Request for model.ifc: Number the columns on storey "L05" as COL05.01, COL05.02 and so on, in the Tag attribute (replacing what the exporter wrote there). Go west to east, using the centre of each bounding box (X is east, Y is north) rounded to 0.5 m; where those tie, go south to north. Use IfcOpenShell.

First a look at what the model holds.

```python
import ifcopenshell
import ifcopenshell.util.element
import ifcopenshell.util.placement

model = ifcopenshell.open("model.ifc")
print(model.schema)
storey = next(s for s in model.by_type("IfcBuildingStorey") if s.Name == "L05")
columns = [e for e in ifcopenshell.util.element.get_decomposition(storey) if e.is_a("IfcColumn")]
for e in sorted(columns, key=lambda e: e.id()):
    origin = ifcopenshell.util.placement.get_local_placement(e.ObjectPlacement)[:3, 3]
    print(e.id(), e.Tag, e.Name, origin.round(2) + 0.0, sep=" | ")
```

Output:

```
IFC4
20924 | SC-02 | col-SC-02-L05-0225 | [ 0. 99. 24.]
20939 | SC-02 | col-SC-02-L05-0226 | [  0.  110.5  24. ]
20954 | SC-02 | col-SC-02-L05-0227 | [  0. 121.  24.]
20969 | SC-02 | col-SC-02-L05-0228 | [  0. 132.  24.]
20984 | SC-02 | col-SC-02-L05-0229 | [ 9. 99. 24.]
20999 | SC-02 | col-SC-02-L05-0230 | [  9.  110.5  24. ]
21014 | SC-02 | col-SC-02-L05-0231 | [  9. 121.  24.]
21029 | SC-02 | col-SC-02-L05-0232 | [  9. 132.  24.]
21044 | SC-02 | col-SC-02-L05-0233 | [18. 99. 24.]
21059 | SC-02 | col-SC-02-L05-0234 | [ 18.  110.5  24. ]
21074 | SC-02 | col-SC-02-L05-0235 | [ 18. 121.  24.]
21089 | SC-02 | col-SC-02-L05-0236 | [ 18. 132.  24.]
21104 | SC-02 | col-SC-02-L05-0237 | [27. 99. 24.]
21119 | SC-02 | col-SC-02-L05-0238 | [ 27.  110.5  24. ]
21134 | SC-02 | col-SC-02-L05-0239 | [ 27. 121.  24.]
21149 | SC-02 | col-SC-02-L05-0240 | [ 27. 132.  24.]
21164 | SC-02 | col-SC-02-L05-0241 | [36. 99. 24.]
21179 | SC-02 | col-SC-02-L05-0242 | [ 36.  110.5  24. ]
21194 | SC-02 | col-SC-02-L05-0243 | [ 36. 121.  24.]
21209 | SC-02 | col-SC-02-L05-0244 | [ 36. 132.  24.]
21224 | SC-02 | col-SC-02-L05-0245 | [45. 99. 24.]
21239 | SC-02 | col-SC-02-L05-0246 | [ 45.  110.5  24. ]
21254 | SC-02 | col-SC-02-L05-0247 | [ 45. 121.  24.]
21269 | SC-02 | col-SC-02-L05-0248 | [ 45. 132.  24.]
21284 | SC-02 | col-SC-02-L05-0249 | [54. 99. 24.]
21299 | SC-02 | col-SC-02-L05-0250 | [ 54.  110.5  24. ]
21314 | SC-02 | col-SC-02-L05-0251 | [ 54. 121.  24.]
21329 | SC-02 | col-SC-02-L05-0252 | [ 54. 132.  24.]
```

```python
import ifcopenshell
import ifcopenshell.geom
import ifcopenshell.util.element
import ifcopenshell.util.shape

model = ifcopenshell.open("model.ifc")
settings = ifcopenshell.geom.settings()
settings.set("use-world-coords", True)


def centre(element):
    shape = ifcopenshell.geom.create_shape(settings, element)
    return ifcopenshell.util.shape.get_bbox_centroid(shape.geometry)


storey = next(s for s in model.by_type("IfcBuildingStorey") if s.Name == "L05")
columns = [e for e in ifcopenshell.util.element.get_decomposition(storey) if e.is_a("IfcColumn")]

# Insertion points can sit at a corner or the storey origin, so sort by the geometry (in metres).
centres = {e: centre(e) for e in columns}
columns.sort(key=lambda e: (round(centres[e][0] / 0.5), centres[e][1]))

for i, e in enumerate(columns, start=1):
    number = f"COL05.{i:02d}"
    e.Tag = number
    print(e.id(), number)

model.write("model_edited.ifc")
```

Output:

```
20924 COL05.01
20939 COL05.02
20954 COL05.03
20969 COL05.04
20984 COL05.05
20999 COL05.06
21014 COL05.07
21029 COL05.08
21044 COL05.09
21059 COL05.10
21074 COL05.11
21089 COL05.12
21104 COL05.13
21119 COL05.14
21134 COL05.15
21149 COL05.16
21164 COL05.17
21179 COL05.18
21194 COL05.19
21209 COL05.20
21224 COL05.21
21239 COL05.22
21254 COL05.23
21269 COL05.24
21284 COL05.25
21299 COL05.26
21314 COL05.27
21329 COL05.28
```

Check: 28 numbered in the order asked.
